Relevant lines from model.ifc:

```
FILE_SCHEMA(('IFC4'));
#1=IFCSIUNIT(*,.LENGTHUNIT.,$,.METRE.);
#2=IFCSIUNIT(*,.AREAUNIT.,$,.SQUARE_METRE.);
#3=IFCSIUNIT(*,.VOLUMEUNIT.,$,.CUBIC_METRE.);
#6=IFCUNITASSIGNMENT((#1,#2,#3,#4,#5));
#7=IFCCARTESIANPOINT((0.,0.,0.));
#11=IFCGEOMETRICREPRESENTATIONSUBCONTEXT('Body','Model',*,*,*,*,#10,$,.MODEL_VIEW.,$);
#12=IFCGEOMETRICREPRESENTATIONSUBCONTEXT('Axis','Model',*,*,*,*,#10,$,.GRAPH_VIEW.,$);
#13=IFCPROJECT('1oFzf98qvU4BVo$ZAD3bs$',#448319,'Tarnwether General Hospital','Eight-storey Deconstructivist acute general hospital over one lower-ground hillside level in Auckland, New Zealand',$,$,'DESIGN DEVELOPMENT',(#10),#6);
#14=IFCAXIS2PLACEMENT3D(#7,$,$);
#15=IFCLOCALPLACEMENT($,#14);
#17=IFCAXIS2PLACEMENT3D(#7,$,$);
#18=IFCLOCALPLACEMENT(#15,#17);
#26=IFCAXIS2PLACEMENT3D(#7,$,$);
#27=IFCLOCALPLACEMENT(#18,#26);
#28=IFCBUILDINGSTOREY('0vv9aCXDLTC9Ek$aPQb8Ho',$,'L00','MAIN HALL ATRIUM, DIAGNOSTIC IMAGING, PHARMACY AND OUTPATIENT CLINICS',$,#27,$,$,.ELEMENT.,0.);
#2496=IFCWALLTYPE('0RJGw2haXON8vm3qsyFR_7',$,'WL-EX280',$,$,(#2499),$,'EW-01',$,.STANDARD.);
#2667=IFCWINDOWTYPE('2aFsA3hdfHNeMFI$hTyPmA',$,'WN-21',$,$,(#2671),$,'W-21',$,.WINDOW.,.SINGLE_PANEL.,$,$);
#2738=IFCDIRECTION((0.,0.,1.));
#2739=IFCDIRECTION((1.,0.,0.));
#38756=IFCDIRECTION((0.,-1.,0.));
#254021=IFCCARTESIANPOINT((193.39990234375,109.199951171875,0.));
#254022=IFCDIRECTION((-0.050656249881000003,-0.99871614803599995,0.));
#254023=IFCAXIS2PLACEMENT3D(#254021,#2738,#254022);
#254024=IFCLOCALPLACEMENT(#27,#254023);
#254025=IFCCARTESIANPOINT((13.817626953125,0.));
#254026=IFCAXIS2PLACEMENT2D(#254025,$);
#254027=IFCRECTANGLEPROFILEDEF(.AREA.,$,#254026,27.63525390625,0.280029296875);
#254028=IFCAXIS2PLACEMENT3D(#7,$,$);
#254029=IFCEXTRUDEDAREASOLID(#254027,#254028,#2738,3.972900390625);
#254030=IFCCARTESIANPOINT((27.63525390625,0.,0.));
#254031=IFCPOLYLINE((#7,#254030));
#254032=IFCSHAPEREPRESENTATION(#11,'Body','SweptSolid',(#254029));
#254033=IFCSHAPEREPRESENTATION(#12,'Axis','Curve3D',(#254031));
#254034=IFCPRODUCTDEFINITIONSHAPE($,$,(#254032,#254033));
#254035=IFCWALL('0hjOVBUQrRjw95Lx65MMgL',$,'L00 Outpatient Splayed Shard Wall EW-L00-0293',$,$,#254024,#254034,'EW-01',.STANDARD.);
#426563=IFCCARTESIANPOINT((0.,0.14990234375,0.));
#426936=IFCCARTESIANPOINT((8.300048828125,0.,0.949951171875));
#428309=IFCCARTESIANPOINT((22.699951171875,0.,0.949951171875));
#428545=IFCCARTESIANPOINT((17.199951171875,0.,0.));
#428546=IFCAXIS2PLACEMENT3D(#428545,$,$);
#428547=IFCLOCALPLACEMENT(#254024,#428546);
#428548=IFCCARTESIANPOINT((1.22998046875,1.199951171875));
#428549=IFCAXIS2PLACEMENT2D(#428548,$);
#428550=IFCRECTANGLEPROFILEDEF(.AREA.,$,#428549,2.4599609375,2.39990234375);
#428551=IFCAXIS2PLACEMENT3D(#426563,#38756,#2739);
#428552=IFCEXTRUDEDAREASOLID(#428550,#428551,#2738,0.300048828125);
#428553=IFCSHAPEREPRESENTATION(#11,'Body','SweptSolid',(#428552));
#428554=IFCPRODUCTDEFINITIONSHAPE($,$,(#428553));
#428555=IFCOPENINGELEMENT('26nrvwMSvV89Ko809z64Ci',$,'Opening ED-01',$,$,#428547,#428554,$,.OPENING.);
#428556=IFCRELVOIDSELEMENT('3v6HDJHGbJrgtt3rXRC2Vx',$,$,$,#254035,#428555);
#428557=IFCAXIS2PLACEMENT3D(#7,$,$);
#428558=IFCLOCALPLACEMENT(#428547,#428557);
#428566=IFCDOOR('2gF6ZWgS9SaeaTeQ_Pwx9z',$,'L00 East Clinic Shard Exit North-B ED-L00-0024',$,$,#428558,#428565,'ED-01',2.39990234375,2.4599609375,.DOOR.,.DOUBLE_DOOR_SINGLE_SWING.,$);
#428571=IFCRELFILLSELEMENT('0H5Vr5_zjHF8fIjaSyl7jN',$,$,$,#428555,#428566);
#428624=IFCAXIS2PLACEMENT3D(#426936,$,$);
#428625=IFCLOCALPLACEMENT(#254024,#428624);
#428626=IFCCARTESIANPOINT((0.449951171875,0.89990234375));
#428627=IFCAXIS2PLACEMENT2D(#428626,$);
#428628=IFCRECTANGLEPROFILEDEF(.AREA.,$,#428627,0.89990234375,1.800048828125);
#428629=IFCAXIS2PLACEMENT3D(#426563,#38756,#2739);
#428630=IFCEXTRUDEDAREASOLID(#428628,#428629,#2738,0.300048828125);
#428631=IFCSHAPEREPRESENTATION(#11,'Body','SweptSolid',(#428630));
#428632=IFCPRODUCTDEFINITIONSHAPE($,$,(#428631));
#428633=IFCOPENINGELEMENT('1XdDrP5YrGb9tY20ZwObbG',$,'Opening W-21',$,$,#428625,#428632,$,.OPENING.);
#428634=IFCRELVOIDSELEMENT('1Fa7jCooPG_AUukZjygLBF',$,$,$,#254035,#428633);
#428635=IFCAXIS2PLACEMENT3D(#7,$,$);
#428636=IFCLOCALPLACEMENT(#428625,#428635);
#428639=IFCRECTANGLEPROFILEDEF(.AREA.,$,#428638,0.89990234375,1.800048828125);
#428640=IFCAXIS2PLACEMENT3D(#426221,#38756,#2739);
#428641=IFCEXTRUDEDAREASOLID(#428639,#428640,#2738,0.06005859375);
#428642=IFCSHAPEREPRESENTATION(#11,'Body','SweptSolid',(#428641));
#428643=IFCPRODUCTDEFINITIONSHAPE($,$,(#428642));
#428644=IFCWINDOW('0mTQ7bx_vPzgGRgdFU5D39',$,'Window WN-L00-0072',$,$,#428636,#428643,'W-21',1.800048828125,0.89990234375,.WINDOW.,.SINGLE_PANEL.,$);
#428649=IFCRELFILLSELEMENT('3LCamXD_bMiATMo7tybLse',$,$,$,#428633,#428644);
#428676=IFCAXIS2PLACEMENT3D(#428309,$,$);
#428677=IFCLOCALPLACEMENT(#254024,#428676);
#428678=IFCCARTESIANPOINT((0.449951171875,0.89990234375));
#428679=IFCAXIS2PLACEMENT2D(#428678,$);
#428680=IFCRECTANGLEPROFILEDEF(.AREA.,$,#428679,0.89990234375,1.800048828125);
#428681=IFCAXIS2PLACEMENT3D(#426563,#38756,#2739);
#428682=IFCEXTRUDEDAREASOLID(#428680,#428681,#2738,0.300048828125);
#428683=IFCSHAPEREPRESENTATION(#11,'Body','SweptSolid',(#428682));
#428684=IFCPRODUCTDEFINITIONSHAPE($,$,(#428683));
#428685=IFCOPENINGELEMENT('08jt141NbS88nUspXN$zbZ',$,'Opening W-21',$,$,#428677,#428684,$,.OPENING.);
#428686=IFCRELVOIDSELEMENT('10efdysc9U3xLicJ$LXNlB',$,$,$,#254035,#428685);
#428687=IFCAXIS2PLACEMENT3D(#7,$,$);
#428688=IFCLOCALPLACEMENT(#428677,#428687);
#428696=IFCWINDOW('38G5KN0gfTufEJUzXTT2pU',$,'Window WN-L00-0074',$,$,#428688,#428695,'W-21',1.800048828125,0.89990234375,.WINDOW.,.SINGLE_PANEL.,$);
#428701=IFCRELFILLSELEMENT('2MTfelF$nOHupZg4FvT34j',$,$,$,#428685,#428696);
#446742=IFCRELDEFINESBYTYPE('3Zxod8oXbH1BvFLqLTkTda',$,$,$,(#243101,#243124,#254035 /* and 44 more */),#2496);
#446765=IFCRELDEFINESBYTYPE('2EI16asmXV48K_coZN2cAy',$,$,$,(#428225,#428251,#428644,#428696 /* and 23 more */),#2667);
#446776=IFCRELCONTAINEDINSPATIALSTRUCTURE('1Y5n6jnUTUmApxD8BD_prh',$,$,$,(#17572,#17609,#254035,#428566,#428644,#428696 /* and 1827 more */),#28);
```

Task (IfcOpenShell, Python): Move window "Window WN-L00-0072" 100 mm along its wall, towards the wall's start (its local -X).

```python
import ifcopenshell
import ifcopenshell.api.geometry
import ifcopenshell.util.placement
import ifcopenshell.util.unit

model = ifcopenshell.open("model.ifc")
unit_scale = ifcopenshell.util.unit.calculate_unit_scale(model)

window = model.by_guid("0mTQ7bx_vPzgGRgdFU5D39")
opening = window.FillsVoids[0].RelatingOpeningElement
wall = opening.VoidsElements[0].RelatingBuildingElement

wall_matrix = ifcopenshell.util.placement.get_local_placement(wall.ObjectPlacement)
shift = wall_matrix[:3, 0] * -0.1 / unit_scale
before = ifcopenshell.util.placement.get_local_placement(window.ObjectPlacement)[:3, 3].copy()

# The window is placed relative to its opening, so it follows when the opening moves.
matrix = ifcopenshell.util.placement.get_local_placement(opening.ObjectPlacement)
matrix[:3, 3] += shift
ifcopenshell.api.geometry.edit_object_placement(
    model, product=opening, matrix=matrix, is_si=False, should_transform_children=True
)

after = ifcopenshell.util.placement.get_local_placement(window.ObjectPlacement)[:3, 3]
print("window moved by", (after - before).round(3) + 0.0)

model.write("model_v2.ifc")
```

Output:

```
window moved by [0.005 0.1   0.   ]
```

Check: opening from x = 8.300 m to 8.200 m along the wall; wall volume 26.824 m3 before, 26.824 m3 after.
